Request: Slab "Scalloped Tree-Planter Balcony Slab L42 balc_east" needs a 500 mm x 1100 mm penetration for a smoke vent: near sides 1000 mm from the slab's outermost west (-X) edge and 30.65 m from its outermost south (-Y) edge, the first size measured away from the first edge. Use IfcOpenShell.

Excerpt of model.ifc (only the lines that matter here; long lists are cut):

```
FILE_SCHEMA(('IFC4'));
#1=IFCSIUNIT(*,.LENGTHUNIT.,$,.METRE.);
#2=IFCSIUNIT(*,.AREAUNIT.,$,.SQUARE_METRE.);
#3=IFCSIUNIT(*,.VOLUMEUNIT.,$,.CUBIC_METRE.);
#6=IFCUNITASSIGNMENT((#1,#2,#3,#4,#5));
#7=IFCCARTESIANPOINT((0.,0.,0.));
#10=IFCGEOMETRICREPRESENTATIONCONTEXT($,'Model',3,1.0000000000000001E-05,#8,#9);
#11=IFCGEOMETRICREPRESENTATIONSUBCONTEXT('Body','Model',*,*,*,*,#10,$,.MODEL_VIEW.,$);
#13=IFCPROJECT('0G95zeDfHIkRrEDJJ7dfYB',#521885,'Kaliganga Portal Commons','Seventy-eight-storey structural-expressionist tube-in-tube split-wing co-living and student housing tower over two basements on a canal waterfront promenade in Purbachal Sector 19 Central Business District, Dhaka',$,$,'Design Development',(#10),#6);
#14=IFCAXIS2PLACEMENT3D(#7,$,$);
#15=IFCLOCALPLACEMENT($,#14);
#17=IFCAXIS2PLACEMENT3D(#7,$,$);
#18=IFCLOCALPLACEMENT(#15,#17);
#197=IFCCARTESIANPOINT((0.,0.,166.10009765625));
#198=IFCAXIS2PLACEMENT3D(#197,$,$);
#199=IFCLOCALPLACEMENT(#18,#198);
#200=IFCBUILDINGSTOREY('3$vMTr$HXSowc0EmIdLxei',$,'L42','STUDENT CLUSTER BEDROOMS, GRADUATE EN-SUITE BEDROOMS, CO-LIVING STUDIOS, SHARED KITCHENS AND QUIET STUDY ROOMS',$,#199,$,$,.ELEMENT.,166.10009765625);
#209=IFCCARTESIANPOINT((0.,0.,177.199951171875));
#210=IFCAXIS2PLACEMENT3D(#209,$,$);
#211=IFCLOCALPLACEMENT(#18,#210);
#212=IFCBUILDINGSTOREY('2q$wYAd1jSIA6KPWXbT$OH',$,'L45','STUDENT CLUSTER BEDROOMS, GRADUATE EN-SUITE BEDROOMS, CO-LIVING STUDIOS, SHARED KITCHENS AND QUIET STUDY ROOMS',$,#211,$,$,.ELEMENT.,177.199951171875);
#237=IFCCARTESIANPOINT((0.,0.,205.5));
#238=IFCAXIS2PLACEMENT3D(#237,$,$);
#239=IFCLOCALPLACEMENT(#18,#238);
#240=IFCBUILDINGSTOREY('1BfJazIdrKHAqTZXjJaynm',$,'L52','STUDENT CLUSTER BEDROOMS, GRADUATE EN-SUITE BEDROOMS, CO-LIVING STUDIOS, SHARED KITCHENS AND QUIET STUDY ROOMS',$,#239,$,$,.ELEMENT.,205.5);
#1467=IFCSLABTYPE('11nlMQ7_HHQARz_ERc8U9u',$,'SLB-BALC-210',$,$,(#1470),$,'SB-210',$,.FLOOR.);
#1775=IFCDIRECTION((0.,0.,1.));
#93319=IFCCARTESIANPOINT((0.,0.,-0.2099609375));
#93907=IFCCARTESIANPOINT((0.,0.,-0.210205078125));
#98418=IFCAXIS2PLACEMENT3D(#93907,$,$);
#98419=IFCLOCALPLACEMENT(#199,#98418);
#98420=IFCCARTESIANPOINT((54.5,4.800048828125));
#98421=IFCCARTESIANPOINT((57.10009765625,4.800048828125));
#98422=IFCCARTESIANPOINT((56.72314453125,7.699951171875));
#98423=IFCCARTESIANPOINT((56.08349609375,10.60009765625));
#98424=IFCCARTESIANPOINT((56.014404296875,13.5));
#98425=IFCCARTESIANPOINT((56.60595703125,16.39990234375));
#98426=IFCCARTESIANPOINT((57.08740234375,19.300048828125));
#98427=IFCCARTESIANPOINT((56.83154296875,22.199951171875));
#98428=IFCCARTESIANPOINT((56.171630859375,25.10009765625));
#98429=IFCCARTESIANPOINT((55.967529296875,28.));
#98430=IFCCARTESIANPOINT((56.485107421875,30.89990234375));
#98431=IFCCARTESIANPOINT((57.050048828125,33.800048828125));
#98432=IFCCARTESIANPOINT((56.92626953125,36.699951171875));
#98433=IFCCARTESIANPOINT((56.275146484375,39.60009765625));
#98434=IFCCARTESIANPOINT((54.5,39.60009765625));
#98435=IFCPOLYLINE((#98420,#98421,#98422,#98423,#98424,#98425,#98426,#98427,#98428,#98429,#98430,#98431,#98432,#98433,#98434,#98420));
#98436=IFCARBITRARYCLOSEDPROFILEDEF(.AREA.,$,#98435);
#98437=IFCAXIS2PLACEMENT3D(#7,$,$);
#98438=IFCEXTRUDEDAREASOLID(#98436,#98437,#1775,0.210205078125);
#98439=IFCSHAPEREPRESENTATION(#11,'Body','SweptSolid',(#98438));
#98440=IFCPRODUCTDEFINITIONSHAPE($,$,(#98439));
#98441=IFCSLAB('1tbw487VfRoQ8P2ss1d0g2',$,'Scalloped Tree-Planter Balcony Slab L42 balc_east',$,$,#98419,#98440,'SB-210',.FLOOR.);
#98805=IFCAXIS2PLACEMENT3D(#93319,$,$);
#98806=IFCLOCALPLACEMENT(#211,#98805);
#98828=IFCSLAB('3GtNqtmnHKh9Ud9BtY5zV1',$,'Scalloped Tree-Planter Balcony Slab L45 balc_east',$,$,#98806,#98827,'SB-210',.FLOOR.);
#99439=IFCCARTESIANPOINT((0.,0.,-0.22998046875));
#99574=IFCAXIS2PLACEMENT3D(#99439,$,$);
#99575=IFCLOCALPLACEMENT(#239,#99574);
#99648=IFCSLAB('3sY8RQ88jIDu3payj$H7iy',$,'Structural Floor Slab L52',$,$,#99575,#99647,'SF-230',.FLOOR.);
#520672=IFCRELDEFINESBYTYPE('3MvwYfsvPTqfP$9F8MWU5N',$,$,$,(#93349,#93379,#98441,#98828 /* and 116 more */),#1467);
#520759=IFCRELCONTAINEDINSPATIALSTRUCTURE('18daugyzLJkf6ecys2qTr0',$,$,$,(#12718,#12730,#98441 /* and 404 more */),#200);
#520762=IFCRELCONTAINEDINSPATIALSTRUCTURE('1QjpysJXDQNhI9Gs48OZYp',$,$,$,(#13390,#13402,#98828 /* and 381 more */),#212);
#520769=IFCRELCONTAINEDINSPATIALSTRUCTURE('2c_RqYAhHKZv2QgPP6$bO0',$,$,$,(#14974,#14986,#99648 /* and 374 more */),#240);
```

```python
import numpy as np
import ifcopenshell
import ifcopenshell.api.feature
import ifcopenshell.api.geometry
import ifcopenshell.api.root
import ifcopenshell.geom
import ifcopenshell.util.placement
import ifcopenshell.util.representation
import ifcopenshell.util.shape
import ifcopenshell.util.unit

model = ifcopenshell.open("model.ifc")
unit_scale = ifcopenshell.util.unit.calculate_unit_scale(model)
settings = ifcopenshell.geom.settings()


def volume(element):
    """Net volume in cubic metres, openings subtracted."""
    shape = ifcopenshell.geom.create_shape(settings, element)
    return ifcopenshell.util.shape.get_volume(shape.geometry)


slab = model.by_guid("1tbw487VfRoQ8P2ss1d0g2")
before = volume(slab)

# Extent in the slab's own axes, in metres. The edges named are its -X and -Y sides.
slab_shape = ifcopenshell.geom.create_shape(settings, slab)
vertices = ifcopenshell.util.shape.get_vertices(slab_shape.geometry)
x_min, y_min, bottom = vertices.min(axis=0)
top = vertices[:, 2].max()

opening = ifcopenshell.api.root.create_entity(model, ifc_class="IfcOpeningElement", name="Smoke vent opening", predefined_type="OPENING")
context = ifcopenshell.util.representation.get_context(model, "Model", "Body", "MODEL_VIEW")
width, depth = 0.5, 1.1
outline = [(0.0, 0.0), (width, 0.0), (width, depth), (0.0, depth), (0.0, 0.0)]
# Overshoot both faces by 50 mm so the cut is clean.
shape = ifcopenshell.api.geometry.add_slab_representation(
    model, context=context, depth=top - bottom + 0.1, polyline=outline
)
ifcopenshell.api.geometry.assign_representation(model, product=opening, representation=shape)

matrix = ifcopenshell.util.placement.get_local_placement(slab.ObjectPlacement)
matrix[:, 3] = matrix @ np.append(np.array([x_min + 1, y_min + 30.65, bottom - 0.05]) / unit_scale, 1.0)
ifcopenshell.api.geometry.edit_object_placement(model, product=opening, matrix=matrix, is_si=False)
ifcopenshell.api.feature.add_feature(model, feature=opening, element=slab)

after = volume(slab)

print(f"slab volume {before:.3f} -> {after:.3f} m3")

model.write("model_rev.ifc")
```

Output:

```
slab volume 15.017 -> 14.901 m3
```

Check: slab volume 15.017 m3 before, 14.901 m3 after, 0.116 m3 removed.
